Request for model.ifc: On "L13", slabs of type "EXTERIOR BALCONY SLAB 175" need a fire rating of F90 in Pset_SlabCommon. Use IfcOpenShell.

First a look at what the model holds.

```python
import ifcopenshell
import ifcopenshell.util.element

model = ifcopenshell.open("model.ifc")
print(model.schema)
storey = next(s for s in model.by_type("IfcBuildingStorey") if s.Name == "L13")
slabs = [e for e in ifcopenshell.util.element.get_decomposition(storey) if e.is_a("IfcSlab")]
seen = {}
for e in slabs:
    element_type = ifcopenshell.util.element.get_type(e)
    key = (element_type.Name if element_type != e and element_type else None, ifcopenshell.util.element.get_pset(e, "Pset_SlabCommon", "FireRating"))
    seen[key] = seen.get(key, 0) + 1
for (name, value), count in sorted(seen.items(), key=str):
    print(count, "x", name, "|", value)
```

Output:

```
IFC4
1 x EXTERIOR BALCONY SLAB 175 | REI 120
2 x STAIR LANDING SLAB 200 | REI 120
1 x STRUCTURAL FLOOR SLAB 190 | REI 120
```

```python
import ifcopenshell
import ifcopenshell.api.pset
import ifcopenshell.util.element

model = ifcopenshell.open("model.ifc")

storey = next(s for s in model.by_type("IfcBuildingStorey") if s.Name == "L13")
slabs = [e for e in ifcopenshell.util.element.get_decomposition(storey) if e.is_a("IfcSlab")]

count = 0
for e in slabs:
    element_type = ifcopenshell.util.element.get_type(e)
    if element_type in (None, e) or element_type.Name != "EXTERIOR BALCONY SLAB 175":
        continue
    found = ifcopenshell.util.element.get_pset(e, "Pset_SlabCommon", should_inherit=False)
    if found:
        pset = model.by_id(found["id"])
        if len(ifcopenshell.util.element.get_elements_by_pset(pset)) > 1:
            pset = ifcopenshell.api.pset.unshare_pset(model, products=[e], pset=pset)[0]
    else:
        pset = ifcopenshell.api.pset.add_pset(model, product=e, name="Pset_SlabCommon")
    ifcopenshell.api.pset.edit_pset(model, pset=pset, properties={"FireRating": "F90"})
    count += 1

print(count, "slabs updated")

model.write("model_rev.ifc")
```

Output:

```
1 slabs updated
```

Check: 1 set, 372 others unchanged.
